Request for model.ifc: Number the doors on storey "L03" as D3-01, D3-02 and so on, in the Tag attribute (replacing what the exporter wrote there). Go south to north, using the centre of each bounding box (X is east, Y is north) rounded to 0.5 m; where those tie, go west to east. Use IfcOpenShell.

First a look at what the model holds.

```python
import ifcopenshell
import ifcopenshell.util.element
import ifcopenshell.util.placement

model = ifcopenshell.open("model.ifc")
print(model.schema)
storey = next(s for s in model.by_type("IfcBuildingStorey") if s.Name == "L03")
doors = [e for e in ifcopenshell.util.element.get_decomposition(storey) if e.is_a("IfcDoor")]
for e in sorted(doors, key=lambda e: e.id()):
    origin = ifcopenshell.util.placement.get_local_placement(e.ObjectPlacement)[:3, 3]
    print(e.id(), e.Tag, e.Name, origin.round(2) + 0.0, sep=" | ")
```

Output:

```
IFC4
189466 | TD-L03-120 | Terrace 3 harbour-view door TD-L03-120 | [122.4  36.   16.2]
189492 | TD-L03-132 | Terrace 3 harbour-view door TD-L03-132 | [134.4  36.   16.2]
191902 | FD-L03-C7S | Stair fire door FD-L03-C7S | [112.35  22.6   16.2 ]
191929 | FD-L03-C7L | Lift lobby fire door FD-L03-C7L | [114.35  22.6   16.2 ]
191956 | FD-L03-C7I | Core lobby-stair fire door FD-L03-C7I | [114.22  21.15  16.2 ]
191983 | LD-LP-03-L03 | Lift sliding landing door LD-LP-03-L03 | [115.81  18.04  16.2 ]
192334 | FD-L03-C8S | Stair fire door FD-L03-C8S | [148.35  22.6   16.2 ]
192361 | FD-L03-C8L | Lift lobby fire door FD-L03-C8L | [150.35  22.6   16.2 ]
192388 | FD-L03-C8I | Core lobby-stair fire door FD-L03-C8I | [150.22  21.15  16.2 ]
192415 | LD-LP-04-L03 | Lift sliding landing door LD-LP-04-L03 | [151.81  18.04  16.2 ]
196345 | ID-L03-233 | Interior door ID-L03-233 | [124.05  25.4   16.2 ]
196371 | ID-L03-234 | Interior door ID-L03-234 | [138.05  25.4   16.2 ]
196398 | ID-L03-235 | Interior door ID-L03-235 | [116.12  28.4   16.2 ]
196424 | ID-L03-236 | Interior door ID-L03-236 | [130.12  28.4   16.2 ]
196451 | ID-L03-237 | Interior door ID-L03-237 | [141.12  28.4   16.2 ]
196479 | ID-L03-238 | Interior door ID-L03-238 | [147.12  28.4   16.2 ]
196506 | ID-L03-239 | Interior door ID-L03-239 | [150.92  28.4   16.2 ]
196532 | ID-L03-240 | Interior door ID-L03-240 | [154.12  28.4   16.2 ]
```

```python
import ifcopenshell
import ifcopenshell.geom
import ifcopenshell.util.element
import ifcopenshell.util.shape

model = ifcopenshell.open("model.ifc")
settings = ifcopenshell.geom.settings()
settings.set("use-world-coords", True)


def centre(element):
    shape = ifcopenshell.geom.create_shape(settings, element)
    return ifcopenshell.util.shape.get_bbox_centroid(shape.geometry)


storey = next(s for s in model.by_type("IfcBuildingStorey") if s.Name == "L03")
doors = [e for e in ifcopenshell.util.element.get_decomposition(storey) if e.is_a("IfcDoor")]

# Insertion points can sit at a corner or the storey origin, so sort by the geometry (in metres).
centres = {e: centre(e) for e in doors}
doors.sort(key=lambda e: (round(centres[e][1] / 0.5), centres[e][0]))

for i, e in enumerate(doors, start=1):
    number = f"D3-{i:02d}"
    e.Tag = number
    print(e.id(), number)

model.write("model-out.ifc")
```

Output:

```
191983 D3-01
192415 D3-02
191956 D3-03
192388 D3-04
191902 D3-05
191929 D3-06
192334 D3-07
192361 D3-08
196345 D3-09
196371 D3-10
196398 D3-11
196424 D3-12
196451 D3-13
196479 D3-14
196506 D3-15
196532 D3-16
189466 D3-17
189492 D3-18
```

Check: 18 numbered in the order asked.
